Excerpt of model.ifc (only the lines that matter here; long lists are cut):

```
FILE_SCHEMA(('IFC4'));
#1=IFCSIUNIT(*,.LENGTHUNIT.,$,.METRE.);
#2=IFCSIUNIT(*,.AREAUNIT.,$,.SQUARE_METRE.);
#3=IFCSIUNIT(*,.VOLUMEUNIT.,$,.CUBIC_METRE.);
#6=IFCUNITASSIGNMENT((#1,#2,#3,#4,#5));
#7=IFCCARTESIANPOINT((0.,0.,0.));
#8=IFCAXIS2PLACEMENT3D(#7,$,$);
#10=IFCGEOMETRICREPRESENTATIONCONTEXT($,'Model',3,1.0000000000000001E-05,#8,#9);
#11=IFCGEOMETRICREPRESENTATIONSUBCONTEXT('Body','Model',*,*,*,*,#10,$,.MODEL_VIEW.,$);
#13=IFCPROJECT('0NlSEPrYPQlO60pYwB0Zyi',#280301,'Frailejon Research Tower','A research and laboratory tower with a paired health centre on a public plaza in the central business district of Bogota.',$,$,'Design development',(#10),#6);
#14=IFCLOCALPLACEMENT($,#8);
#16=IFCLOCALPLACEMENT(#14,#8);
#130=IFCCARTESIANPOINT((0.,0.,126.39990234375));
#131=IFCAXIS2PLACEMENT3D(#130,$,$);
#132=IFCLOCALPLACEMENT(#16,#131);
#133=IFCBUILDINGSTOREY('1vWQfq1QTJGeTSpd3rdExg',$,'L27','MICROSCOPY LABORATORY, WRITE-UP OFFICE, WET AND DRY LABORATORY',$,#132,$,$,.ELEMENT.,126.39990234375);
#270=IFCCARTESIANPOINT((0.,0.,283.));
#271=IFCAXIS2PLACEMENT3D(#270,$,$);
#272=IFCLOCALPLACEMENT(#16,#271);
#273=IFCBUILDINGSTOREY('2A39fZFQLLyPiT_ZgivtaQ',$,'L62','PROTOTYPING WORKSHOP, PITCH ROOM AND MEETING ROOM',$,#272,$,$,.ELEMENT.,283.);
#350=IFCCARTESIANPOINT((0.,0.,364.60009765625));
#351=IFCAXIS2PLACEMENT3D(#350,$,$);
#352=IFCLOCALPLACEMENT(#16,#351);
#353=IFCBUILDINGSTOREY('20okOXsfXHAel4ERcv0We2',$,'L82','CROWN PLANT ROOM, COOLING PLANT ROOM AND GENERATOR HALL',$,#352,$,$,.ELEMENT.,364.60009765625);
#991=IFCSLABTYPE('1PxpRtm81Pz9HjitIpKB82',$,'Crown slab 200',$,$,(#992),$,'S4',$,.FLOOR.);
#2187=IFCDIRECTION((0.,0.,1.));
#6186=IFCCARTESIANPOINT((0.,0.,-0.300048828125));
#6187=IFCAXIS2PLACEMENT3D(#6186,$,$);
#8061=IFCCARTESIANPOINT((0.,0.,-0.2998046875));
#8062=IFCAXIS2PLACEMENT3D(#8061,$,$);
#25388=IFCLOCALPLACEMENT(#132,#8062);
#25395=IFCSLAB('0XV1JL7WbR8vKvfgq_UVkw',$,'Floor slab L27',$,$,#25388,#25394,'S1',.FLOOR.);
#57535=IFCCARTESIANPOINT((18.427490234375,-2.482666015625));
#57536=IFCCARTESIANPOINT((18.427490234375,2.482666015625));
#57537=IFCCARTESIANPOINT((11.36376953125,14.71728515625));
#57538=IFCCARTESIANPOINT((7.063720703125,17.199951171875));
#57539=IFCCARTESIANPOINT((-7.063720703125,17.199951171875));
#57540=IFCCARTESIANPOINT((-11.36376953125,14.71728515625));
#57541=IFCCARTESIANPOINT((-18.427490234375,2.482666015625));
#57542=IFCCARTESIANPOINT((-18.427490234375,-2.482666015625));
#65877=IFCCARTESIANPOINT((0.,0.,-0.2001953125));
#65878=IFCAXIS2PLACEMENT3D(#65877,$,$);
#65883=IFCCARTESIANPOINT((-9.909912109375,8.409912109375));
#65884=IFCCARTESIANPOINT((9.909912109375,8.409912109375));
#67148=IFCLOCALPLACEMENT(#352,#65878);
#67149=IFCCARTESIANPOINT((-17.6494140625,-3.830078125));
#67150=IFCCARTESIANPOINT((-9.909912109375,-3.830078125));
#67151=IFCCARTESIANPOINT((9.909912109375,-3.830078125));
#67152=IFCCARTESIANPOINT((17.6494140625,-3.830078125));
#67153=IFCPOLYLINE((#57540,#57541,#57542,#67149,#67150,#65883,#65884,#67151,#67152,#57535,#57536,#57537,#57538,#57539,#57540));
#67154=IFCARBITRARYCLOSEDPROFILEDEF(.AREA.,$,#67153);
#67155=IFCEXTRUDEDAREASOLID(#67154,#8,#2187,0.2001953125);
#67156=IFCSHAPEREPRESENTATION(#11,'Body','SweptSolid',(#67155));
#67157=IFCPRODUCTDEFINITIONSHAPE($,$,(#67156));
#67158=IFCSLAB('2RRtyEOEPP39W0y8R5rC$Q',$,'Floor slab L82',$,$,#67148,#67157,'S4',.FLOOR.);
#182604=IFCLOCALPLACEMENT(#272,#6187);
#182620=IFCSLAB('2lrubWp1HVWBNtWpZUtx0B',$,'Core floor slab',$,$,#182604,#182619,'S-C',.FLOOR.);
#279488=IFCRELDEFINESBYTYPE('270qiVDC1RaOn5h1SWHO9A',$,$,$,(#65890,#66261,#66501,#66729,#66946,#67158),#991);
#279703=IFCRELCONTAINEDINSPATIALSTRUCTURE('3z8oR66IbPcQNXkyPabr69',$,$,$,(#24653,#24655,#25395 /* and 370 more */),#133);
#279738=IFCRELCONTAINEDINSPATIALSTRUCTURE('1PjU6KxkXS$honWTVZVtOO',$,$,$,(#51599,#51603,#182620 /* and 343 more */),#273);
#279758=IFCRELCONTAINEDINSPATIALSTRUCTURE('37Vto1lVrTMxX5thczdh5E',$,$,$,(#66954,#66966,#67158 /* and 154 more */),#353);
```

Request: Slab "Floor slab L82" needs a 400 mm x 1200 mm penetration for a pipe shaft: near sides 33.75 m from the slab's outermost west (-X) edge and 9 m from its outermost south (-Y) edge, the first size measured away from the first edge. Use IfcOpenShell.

```python
import numpy as np
import ifcopenshell
import ifcopenshell.api.feature
import ifcopenshell.api.geometry
import ifcopenshell.api.root
import ifcopenshell.geom
import ifcopenshell.util.placement
import ifcopenshell.util.representation
import ifcopenshell.util.shape
import ifcopenshell.util.unit

model = ifcopenshell.open("model.ifc")
unit_scale = ifcopenshell.util.unit.calculate_unit_scale(model)
settings = ifcopenshell.geom.settings()


def volume(element):
    """Net volume in cubic metres, openings subtracted."""
    shape = ifcopenshell.geom.create_shape(settings, element)
    return ifcopenshell.util.shape.get_volume(shape.geometry)


slab = model.by_id(67158)
before = volume(slab)

# Extent in the slab's own axes, in metres. The edges named are its -X and -Y sides.
slab_shape = ifcopenshell.geom.create_shape(settings, slab)
vertices = ifcopenshell.util.shape.get_vertices(slab_shape.geometry)
x_min, y_min, bottom = vertices.min(axis=0)
top = vertices[:, 2].max()

opening = ifcopenshell.api.root.create_entity(model, ifc_class="IfcOpeningElement", name="Pipe shaft opening", predefined_type="OPENING")
context = ifcopenshell.util.representation.get_context(model, "Model", "Body", "MODEL_VIEW")
width, depth = 0.4, 1.2
outline = [(0.0, 0.0), (width, 0.0), (width, depth), (0.0, depth), (0.0, 0.0)]
# Overshoot both faces by 50 mm so the cut is clean.
shape = ifcopenshell.api.geometry.add_slab_representation(
    model, context=context, depth=top - bottom + 0.1, polyline=outline
)
ifcopenshell.api.geometry.assign_representation(model, product=opening, representation=shape)

matrix = ifcopenshell.util.placement.get_local_placement(slab.ObjectPlacement)
matrix[:, 3] = matrix @ np.append(np.array([x_min + 33.75, y_min + 9, bottom - 0.05]) / unit_scale, 1.0)
ifcopenshell.api.geometry.edit_object_placement(model, product=opening, matrix=matrix, is_si=False)
ifcopenshell.api.feature.add_feature(model, feature=opening, element=slab)

after = volume(slab)

print(f"slab volume {before:.3f} -> {after:.3f} m3")

model.write("model_rev.ifc")
```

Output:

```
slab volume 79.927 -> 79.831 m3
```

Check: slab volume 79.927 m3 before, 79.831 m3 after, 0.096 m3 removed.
